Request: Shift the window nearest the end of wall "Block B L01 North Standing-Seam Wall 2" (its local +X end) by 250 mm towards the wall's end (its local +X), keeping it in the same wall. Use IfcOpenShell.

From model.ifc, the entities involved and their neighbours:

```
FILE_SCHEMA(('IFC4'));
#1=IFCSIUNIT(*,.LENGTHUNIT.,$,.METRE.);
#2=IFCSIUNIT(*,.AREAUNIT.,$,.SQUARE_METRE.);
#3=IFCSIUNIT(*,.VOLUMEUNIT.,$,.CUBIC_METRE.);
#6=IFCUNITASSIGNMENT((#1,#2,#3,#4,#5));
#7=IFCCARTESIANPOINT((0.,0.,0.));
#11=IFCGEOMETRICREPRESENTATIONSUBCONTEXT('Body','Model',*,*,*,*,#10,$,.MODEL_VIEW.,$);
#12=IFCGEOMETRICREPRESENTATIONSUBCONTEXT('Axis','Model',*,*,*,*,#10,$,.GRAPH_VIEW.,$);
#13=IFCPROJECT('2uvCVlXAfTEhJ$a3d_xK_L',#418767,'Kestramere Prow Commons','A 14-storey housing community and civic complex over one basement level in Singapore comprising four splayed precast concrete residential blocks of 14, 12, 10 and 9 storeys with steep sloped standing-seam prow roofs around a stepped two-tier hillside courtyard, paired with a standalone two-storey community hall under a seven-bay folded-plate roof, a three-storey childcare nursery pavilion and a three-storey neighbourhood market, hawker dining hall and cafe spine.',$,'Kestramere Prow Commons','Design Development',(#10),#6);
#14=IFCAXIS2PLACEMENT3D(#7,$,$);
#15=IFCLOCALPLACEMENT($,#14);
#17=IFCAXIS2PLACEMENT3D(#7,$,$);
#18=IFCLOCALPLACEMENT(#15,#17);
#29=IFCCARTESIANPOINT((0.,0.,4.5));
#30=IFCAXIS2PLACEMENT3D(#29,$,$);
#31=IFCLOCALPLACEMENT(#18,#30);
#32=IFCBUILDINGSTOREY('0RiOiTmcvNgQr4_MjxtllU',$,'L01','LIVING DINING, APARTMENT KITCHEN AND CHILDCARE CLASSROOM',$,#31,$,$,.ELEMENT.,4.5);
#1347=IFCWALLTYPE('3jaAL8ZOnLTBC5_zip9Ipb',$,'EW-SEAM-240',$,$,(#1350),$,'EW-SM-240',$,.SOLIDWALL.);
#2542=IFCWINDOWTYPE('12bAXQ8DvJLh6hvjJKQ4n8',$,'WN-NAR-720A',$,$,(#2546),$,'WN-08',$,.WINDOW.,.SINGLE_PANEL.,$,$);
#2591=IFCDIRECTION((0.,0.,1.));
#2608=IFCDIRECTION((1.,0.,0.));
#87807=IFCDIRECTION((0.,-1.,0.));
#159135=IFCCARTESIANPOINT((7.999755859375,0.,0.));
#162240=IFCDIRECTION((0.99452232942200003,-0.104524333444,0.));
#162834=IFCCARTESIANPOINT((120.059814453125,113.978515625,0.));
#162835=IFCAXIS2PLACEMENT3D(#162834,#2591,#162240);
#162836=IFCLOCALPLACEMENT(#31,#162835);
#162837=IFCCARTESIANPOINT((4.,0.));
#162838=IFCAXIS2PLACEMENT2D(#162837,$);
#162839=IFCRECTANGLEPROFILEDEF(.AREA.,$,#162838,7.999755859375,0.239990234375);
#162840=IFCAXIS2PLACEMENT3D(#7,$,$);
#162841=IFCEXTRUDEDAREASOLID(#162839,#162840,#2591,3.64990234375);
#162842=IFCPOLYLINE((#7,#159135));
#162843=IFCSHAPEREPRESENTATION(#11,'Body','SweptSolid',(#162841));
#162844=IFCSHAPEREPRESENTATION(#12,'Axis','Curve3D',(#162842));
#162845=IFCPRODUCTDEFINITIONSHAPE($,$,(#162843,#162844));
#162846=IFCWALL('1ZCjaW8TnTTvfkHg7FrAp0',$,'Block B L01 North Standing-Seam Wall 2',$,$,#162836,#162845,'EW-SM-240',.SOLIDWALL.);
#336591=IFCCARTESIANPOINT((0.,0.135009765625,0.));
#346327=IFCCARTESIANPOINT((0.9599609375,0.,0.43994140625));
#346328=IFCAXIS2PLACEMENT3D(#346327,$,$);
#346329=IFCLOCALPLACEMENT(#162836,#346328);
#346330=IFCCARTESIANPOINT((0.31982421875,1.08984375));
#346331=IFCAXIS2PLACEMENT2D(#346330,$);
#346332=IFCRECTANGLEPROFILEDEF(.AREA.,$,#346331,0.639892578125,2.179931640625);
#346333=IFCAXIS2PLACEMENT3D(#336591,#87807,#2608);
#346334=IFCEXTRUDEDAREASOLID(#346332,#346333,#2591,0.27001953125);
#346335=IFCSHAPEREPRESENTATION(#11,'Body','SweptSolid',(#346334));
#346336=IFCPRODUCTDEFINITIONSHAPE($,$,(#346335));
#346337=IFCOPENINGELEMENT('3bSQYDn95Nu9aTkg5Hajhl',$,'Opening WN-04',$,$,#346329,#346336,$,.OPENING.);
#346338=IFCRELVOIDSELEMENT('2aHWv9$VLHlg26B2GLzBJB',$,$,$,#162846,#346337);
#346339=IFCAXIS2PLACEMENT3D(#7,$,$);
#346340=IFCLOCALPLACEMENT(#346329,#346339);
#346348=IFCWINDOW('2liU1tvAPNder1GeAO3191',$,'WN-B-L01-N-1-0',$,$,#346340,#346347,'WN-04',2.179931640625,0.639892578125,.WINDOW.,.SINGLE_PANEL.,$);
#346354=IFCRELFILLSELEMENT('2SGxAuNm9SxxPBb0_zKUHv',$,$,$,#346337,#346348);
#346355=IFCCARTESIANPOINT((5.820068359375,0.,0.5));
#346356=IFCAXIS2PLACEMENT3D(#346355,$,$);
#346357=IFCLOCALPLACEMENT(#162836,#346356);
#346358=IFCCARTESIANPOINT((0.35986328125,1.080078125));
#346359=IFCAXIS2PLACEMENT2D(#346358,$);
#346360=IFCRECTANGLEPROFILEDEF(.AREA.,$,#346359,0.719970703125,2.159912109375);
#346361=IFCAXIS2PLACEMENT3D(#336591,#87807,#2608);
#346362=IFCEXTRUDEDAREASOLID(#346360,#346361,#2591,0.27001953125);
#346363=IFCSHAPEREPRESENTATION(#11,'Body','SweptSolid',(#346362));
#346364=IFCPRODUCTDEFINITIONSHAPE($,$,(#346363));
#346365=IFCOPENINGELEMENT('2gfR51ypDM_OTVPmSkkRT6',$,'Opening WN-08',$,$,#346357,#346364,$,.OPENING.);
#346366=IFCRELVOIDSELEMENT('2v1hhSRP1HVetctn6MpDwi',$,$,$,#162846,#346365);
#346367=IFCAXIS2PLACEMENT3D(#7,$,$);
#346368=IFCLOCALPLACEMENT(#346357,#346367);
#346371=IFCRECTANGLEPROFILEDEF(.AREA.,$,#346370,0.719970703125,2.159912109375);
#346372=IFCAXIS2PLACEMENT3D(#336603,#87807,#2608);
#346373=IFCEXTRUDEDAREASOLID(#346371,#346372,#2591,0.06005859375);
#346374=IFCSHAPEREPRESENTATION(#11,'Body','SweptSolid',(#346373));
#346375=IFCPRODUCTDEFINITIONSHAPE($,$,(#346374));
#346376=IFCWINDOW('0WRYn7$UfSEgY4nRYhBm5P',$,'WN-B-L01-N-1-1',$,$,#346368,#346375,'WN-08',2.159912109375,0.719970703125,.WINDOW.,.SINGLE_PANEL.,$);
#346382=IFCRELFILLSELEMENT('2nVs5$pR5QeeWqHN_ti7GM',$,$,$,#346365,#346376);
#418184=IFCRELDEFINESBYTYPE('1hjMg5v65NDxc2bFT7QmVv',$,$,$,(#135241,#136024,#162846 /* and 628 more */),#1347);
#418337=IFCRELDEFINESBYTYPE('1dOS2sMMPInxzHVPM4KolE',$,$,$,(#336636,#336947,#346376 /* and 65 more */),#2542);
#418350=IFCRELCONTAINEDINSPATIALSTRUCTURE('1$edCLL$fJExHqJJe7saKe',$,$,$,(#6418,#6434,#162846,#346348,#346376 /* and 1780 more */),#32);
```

```python
import ifcopenshell
import ifcopenshell.api.geometry
import ifcopenshell.util.placement

model = ifcopenshell.open("model.ifc")

window = model.by_guid("0WRYn7$UfSEgY4nRYhBm5P")
opening = window.FillsVoids[0].RelatingOpeningElement
wall = opening.VoidsElements[0].RelatingBuildingElement

wall_matrix = ifcopenshell.util.placement.get_local_placement(wall.ObjectPlacement)
shift = wall_matrix[:3, 0] * 0.25
before = ifcopenshell.util.placement.get_local_placement(window.ObjectPlacement)[:3, 3].copy()

# The window is placed relative to its opening, so it follows when the opening moves.
matrix = ifcopenshell.util.placement.get_local_placement(opening.ObjectPlacement)
matrix[:3, 3] += shift
ifcopenshell.api.geometry.edit_object_placement(
    model, product=opening, matrix=matrix, is_si=False, should_transform_children=True
)

after = ifcopenshell.util.placement.get_local_placement(window.ObjectPlacement)[:3, 3]
print("window moved by", (after - before).round(3) + 0.0)

model.write("model-out.ifc")
```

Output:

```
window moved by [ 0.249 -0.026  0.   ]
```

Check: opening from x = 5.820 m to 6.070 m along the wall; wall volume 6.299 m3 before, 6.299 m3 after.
